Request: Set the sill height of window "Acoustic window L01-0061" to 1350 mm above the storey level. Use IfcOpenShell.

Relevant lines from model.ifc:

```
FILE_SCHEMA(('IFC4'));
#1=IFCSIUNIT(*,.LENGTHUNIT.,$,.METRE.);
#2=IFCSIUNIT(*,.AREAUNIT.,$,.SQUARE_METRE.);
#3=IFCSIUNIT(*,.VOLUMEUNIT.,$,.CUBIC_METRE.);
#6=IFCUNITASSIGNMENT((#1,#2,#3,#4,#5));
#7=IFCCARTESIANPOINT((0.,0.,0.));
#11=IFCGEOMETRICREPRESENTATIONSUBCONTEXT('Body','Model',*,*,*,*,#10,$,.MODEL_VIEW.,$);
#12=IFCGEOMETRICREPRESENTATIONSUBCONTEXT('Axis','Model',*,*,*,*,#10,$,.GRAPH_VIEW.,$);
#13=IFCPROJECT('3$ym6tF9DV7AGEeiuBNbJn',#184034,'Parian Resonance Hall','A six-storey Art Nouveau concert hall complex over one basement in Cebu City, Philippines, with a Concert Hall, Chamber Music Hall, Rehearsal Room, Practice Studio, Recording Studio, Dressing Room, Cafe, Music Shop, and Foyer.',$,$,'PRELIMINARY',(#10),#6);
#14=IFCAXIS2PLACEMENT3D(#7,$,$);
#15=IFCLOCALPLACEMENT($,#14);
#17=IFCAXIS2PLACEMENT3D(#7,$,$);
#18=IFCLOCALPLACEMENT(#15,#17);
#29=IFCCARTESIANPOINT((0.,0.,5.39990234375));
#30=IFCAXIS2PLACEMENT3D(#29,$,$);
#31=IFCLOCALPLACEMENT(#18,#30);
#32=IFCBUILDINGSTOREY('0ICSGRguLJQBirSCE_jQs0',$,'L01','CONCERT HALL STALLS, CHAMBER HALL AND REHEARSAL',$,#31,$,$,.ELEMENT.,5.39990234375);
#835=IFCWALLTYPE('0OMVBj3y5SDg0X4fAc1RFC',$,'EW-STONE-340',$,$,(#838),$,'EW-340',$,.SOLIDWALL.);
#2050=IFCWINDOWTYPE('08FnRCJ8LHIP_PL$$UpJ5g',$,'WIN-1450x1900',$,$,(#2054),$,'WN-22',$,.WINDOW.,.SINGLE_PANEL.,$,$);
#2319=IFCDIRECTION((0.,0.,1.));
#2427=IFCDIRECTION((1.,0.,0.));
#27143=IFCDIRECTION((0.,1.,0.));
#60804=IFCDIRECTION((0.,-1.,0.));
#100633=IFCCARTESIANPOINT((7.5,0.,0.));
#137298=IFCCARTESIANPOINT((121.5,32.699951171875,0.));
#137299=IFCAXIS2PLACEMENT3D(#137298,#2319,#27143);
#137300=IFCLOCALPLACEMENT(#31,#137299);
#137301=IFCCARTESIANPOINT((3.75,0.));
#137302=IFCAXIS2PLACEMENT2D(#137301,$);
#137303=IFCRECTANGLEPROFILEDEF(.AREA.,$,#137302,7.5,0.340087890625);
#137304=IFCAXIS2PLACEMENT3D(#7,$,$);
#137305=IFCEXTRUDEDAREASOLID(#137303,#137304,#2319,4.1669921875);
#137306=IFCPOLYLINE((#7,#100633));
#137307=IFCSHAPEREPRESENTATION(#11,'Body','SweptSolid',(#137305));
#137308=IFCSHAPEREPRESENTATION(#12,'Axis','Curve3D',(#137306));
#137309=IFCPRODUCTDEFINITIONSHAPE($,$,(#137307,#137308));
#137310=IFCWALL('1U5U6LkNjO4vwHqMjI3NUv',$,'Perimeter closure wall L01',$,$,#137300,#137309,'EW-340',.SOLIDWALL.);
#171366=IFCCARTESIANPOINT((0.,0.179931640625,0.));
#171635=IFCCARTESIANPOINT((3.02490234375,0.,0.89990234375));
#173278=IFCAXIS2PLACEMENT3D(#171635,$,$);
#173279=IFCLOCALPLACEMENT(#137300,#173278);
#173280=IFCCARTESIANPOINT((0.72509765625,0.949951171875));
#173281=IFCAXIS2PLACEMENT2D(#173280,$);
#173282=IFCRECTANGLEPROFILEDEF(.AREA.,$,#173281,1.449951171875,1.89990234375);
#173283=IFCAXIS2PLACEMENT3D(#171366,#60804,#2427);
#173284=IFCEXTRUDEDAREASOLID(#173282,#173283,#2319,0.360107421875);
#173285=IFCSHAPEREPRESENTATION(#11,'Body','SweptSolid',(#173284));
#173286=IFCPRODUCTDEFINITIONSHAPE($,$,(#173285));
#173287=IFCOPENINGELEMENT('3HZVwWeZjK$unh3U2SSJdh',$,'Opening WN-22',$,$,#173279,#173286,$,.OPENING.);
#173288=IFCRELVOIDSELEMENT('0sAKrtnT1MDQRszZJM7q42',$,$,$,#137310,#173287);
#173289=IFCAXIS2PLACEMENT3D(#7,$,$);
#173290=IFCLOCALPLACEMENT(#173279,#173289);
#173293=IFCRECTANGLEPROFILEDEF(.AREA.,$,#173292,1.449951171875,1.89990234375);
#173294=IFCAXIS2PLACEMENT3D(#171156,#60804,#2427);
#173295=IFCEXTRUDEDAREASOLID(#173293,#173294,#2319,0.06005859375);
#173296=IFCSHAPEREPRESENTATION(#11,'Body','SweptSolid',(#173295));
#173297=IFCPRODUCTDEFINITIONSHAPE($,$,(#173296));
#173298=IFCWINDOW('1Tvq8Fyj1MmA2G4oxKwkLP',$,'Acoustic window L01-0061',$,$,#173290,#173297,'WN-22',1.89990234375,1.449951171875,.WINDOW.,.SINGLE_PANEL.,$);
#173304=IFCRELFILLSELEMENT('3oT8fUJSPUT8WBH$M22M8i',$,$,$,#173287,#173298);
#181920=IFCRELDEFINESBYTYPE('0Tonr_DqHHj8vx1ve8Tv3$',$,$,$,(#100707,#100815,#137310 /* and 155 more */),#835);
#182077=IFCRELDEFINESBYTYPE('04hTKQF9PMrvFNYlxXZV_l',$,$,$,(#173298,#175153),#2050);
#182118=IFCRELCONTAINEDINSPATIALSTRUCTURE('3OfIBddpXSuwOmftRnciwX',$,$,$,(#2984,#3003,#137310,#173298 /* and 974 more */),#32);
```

```python
import numpy as np
import ifcopenshell
import ifcopenshell.api.geometry
import ifcopenshell.geom
import ifcopenshell.util.element
import ifcopenshell.util.placement
import ifcopenshell.util.shape
import ifcopenshell.util.unit

model = ifcopenshell.open("model.ifc")
unit_scale = ifcopenshell.util.unit.calculate_unit_scale(model)

window = model.by_guid("1Tvq8Fyj1MmA2G4oxKwkLP")
opening = window.FillsVoids[0].RelatingOpeningElement
storey = ifcopenshell.util.element.get_container(window, ifc_class="IfcBuildingStorey")
level = ifcopenshell.util.placement.get_local_placement(storey.ObjectPlacement)[2, 3]

# The opening's origin need not be at the sill, so measure its lowest point.
shape = ifcopenshell.geom.create_shape(ifcopenshell.geom.settings(), opening)
bottom = ifcopenshell.util.shape.get_shape_bottom_elevation(shape, shape.geometry) / unit_scale
dz = level + 1.35 / unit_scale - bottom

shift = np.array([0.0, 0.0, dz])
# The window is placed relative to its opening, so it follows when the opening moves.
matrix = ifcopenshell.util.placement.get_local_placement(opening.ObjectPlacement)
matrix[:3, 3] += shift
ifcopenshell.api.geometry.edit_object_placement(
    model, product=opening, matrix=matrix, is_si=False, should_transform_children=True
)

print(f"moved by {dz * unit_scale:+.3f} m")

model.write("model_rev.ifc")
```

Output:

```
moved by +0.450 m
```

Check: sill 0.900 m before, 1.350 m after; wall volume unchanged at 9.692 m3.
